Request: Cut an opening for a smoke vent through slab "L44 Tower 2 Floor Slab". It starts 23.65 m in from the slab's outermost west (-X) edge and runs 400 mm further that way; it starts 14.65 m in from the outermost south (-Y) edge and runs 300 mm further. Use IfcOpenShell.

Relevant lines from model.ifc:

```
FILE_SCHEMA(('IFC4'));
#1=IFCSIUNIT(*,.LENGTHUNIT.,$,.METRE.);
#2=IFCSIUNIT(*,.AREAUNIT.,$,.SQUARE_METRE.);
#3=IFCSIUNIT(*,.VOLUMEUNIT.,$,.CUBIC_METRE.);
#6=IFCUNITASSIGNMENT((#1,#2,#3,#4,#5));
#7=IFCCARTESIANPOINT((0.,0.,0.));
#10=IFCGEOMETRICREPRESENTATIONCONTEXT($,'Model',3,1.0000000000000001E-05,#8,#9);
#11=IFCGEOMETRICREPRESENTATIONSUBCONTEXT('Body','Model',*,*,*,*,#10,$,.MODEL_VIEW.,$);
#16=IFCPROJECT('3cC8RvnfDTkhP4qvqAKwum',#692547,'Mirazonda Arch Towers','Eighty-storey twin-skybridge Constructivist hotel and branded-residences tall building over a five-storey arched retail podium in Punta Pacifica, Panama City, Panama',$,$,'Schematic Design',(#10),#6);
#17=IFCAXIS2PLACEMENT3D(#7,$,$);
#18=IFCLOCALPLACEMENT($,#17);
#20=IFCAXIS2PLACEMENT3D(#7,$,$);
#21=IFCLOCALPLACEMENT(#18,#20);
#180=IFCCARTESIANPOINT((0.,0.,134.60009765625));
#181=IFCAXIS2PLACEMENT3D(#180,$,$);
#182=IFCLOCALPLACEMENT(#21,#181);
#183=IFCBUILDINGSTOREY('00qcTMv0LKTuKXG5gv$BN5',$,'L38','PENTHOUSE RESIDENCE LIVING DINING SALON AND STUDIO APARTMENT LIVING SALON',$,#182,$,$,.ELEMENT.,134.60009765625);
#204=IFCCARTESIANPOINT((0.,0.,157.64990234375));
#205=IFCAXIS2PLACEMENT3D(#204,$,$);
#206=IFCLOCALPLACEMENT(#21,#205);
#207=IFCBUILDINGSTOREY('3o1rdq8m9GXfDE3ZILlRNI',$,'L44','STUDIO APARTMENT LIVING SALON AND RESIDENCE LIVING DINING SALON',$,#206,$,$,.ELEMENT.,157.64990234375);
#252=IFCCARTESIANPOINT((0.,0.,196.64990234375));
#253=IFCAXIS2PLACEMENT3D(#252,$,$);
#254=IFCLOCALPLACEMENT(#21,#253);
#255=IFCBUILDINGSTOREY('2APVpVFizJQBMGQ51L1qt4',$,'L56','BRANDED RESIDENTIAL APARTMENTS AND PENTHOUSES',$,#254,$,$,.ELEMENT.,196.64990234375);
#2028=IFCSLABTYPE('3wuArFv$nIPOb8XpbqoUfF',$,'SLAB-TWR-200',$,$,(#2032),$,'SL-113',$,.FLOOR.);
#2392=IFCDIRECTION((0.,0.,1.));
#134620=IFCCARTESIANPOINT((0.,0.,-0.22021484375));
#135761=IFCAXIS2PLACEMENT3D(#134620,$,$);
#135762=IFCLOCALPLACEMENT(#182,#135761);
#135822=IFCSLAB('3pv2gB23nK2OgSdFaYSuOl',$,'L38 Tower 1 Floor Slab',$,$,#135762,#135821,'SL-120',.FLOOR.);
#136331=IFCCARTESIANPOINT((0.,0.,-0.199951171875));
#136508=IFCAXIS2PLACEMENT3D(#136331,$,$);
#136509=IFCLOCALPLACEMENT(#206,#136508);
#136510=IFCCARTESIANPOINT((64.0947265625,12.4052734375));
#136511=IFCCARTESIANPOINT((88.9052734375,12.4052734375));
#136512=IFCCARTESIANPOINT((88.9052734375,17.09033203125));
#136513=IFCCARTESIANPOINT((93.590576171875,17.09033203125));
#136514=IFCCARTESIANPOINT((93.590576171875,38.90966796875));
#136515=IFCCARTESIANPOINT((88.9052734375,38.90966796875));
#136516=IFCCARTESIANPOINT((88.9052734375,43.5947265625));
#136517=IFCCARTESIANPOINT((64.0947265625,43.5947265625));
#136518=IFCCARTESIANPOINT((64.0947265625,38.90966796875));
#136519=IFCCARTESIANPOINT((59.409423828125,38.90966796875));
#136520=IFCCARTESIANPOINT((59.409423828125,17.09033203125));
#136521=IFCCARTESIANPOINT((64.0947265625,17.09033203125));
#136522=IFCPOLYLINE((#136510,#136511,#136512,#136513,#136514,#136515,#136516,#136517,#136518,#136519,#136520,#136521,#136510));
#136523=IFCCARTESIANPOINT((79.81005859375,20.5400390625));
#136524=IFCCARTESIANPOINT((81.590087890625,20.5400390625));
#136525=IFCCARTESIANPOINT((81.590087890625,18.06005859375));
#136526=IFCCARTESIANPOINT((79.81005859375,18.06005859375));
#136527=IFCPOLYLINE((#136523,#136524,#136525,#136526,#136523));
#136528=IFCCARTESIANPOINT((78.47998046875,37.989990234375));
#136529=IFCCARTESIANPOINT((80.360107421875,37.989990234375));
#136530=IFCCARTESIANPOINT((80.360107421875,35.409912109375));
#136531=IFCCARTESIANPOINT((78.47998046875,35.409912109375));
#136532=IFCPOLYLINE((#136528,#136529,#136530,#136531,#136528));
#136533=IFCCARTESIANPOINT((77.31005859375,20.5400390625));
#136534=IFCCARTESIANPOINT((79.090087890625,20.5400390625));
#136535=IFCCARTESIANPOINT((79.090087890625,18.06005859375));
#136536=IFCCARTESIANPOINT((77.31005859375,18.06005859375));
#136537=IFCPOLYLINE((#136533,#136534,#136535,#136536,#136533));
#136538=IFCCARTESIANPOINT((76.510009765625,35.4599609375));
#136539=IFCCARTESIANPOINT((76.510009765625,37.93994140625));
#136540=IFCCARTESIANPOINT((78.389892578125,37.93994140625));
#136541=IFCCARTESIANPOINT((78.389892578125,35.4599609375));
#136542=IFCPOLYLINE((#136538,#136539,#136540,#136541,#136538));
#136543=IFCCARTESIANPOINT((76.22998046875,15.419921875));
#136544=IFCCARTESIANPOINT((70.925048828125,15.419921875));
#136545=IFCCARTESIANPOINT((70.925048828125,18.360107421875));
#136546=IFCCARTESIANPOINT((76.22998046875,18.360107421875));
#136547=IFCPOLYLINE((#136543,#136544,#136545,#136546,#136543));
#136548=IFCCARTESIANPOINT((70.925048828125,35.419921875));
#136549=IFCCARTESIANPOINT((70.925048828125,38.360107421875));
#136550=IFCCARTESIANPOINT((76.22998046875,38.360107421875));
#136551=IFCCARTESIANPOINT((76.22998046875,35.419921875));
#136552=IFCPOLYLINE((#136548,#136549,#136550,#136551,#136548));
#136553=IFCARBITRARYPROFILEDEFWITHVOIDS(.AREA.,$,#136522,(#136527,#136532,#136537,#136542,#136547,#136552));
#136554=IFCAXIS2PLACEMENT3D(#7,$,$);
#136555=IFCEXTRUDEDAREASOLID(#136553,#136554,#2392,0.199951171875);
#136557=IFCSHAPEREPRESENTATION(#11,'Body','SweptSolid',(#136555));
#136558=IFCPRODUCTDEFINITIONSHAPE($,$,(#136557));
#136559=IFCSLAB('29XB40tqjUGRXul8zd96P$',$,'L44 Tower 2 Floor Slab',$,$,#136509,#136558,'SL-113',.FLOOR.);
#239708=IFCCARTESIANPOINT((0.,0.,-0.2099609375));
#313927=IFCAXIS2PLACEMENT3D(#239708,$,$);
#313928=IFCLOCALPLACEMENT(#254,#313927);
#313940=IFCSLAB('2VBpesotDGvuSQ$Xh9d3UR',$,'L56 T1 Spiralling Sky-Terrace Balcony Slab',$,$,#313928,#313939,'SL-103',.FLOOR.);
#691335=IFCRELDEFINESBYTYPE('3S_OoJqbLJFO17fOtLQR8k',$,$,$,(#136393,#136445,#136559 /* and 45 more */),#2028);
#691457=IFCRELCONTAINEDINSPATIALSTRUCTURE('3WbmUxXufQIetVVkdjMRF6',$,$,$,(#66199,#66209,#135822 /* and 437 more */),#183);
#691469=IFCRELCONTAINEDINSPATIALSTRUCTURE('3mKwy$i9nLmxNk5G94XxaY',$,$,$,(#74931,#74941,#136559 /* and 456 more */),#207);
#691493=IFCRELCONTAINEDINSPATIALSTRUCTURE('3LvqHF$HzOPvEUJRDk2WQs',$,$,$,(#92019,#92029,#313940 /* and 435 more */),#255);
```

```python
import numpy as np
import ifcopenshell
import ifcopenshell.api.feature
import ifcopenshell.api.geometry
import ifcopenshell.api.root
import ifcopenshell.geom
import ifcopenshell.util.placement
import ifcopenshell.util.representation
import ifcopenshell.util.shape
import ifcopenshell.util.unit

model = ifcopenshell.open("model.ifc")
unit_scale = ifcopenshell.util.unit.calculate_unit_scale(model)
settings = ifcopenshell.geom.settings()


def volume(element):
    """Net volume in cubic metres, openings subtracted."""
    shape = ifcopenshell.geom.create_shape(settings, element)
    return ifcopenshell.util.shape.get_volume(shape.geometry)


slab = model.by_guid("29XB40tqjUGRXul8zd96P$")
before = volume(slab)

# Extent in the slab's own axes, in metres. The edges named are its -X and -Y sides.
slab_shape = ifcopenshell.geom.create_shape(settings, slab)
vertices = ifcopenshell.util.shape.get_vertices(slab_shape.geometry)
x_min, y_min, bottom = vertices.min(axis=0)
top = vertices[:, 2].max()

opening = ifcopenshell.api.root.create_entity(model, ifc_class="IfcOpeningElement", name="Smoke vent opening", predefined_type="OPENING")
context = ifcopenshell.util.representation.get_context(model, "Model", "Body", "MODEL_VIEW")
width, depth = 0.4, 0.3
outline = [(0.0, 0.0), (width, 0.0), (width, depth), (0.0, depth), (0.0, 0.0)]
# Overshoot both faces by 50 mm so the cut is clean.
shape = ifcopenshell.api.geometry.add_slab_representation(
    model, context=context, depth=top - bottom + 0.1, polyline=outline
)
ifcopenshell.api.geometry.assign_representation(model, product=opening, representation=shape)

matrix = ifcopenshell.util.placement.get_local_placement(slab.ObjectPlacement)
matrix[:, 3] = matrix @ np.append(np.array([x_min + 23.65, y_min + 14.65, bottom - 0.05]) / unit_scale, 1.0)
ifcopenshell.api.geometry.edit_object_placement(model, product=opening, matrix=matrix, is_si=False)
ifcopenshell.api.feature.add_feature(model, feature=opening, element=slab)

after = volume(slab)

print(f"slab volume {before:.3f} -> {after:.3f} m3")

model.write("model_edited.ifc")
```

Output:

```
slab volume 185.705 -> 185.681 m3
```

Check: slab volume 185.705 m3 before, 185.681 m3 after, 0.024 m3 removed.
